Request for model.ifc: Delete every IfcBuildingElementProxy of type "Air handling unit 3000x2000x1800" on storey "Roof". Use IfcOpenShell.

First a look at what the model holds.

```python
import ifcopenshell
import ifcopenshell.util.element

model = ifcopenshell.open("model.ifc")
print(model.schema)
storey = next(s for s in model.by_type("IfcBuildingStorey") if s.Name == "Roof")
proxies = [e for e in ifcopenshell.util.element.get_decomposition(storey) if e.is_a("IfcBuildingElementProxy")]
seen = {}
for e in proxies:
    element_type = ifcopenshell.util.element.get_type(e)
    name = element_type.Name if element_type not in (None, e) else None
    seen[name] = seen.get(name, 0) + 1
for name, count in sorted(seen.items(), key=str):
    print(count, "x", name)
```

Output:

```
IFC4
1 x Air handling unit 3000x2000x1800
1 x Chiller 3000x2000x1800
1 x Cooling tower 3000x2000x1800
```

```python
import ifcopenshell
import ifcopenshell.api.root
import ifcopenshell.util.element

model = ifcopenshell.open("model.ifc")

storey = next(s for s in model.by_type("IfcBuildingStorey") if s.Name == "Roof")
proxies = [e for e in ifcopenshell.util.element.get_decomposition(storey) if e.is_a("IfcBuildingElementProxy")]
targets = [e for e in proxies if (t := ifcopenshell.util.element.get_type(e)) not in (None, e) and t.Name == "Air handling unit 3000x2000x1800"]

for e in targets:
    ifcopenshell.api.root.remove_product(model, product=e)
print(len(targets), "removed")

model.write("model_updated.ifc")
```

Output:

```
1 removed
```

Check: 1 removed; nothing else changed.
